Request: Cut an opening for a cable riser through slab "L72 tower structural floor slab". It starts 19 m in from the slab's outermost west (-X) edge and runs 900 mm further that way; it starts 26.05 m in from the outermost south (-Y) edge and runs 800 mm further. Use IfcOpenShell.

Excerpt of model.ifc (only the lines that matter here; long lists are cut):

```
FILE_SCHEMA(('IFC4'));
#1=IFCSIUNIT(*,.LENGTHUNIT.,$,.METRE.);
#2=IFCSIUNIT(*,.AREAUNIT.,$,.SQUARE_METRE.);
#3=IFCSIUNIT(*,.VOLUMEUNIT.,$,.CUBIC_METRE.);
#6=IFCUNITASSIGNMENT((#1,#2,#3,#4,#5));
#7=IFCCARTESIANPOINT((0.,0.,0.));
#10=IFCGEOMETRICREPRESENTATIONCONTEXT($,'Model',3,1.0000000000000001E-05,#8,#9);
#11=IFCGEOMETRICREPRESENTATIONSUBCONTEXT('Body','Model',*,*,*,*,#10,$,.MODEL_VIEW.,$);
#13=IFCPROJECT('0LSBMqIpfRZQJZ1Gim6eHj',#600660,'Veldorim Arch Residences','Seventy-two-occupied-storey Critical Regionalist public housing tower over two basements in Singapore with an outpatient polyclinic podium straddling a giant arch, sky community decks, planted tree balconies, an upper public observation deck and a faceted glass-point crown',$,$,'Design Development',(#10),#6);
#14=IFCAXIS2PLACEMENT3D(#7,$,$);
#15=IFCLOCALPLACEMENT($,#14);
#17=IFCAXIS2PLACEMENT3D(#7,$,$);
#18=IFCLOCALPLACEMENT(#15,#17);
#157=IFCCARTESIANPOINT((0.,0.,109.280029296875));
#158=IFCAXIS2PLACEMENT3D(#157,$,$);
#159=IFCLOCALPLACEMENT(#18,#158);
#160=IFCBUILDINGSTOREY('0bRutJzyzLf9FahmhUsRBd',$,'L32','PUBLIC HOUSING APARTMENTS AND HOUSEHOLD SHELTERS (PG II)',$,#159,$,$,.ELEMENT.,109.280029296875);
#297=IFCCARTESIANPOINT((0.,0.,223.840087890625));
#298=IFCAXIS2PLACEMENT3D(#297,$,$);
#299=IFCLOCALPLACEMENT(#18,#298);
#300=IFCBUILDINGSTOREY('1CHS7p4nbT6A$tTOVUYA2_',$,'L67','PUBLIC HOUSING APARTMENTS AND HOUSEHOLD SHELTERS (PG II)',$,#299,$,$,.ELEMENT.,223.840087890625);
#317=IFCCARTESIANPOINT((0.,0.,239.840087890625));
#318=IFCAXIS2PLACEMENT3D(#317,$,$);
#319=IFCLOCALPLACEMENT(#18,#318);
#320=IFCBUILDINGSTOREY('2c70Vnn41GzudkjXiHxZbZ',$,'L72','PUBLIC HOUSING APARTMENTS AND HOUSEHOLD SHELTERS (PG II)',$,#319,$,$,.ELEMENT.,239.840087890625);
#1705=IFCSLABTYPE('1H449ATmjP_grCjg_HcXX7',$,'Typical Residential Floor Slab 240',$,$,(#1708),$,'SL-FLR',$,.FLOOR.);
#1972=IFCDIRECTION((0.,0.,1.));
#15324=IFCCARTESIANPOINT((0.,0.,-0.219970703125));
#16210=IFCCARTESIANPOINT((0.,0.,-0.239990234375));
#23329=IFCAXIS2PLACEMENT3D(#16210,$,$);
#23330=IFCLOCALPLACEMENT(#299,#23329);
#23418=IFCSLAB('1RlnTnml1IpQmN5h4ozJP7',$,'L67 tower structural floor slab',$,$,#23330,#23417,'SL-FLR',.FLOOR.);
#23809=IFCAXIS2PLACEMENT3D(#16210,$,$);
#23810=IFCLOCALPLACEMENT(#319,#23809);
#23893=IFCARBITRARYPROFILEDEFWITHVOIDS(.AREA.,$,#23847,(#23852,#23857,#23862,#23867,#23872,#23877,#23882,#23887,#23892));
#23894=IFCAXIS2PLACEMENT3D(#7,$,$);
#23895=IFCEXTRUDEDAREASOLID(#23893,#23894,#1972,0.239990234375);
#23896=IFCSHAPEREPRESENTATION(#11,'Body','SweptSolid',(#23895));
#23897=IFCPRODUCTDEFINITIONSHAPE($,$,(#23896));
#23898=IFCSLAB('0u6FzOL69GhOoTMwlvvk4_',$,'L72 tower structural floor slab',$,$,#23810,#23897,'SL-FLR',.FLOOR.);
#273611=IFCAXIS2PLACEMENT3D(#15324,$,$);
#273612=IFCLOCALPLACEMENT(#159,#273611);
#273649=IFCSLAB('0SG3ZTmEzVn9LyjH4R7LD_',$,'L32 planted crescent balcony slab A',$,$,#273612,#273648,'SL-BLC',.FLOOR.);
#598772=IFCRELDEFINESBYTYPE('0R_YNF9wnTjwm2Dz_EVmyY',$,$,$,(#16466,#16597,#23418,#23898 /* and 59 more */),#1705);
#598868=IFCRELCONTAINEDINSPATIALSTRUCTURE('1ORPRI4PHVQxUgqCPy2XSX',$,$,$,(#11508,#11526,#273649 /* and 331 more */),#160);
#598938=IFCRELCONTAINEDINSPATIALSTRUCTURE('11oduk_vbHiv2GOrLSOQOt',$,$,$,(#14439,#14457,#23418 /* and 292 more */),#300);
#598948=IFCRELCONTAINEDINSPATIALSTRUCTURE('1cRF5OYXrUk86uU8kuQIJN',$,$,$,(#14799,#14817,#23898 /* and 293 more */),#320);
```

```python
import numpy as np
import ifcopenshell
import ifcopenshell.api.feature
import ifcopenshell.api.geometry
import ifcopenshell.api.root
import ifcopenshell.geom
import ifcopenshell.util.placement
import ifcopenshell.util.representation
import ifcopenshell.util.shape
import ifcopenshell.util.unit

model = ifcopenshell.open("model.ifc")
unit_scale = ifcopenshell.util.unit.calculate_unit_scale(model)
settings = ifcopenshell.geom.settings()


def volume(element):
    """Net volume in cubic metres, openings subtracted."""
    shape = ifcopenshell.geom.create_shape(settings, element)
    return ifcopenshell.util.shape.get_volume(shape.geometry)


slab = model.by_guid("0u6FzOL69GhOoTMwlvvk4_")
before = volume(slab)

# Extent in the slab's own axes, in metres. The edges named are its -X and -Y sides.
slab_shape = ifcopenshell.geom.create_shape(settings, slab)
vertices = ifcopenshell.util.shape.get_vertices(slab_shape.geometry)
x_min, y_min, bottom = vertices.min(axis=0)
top = vertices[:, 2].max()

opening = ifcopenshell.api.root.create_entity(model, ifc_class="IfcOpeningElement", name="Cable riser opening", predefined_type="OPENING")
context = ifcopenshell.util.representation.get_context(model, "Model", "Body", "MODEL_VIEW")
width, depth = 0.9, 0.8
outline = [(0.0, 0.0), (width, 0.0), (width, depth), (0.0, depth), (0.0, 0.0)]
# Overshoot both faces by 50 mm so the cut is clean.
shape = ifcopenshell.api.geometry.add_slab_representation(
    model, context=context, depth=top - bottom + 0.1, polyline=outline
)
ifcopenshell.api.geometry.assign_representation(model, product=opening, representation=shape)

matrix = ifcopenshell.util.placement.get_local_placement(slab.ObjectPlacement)
matrix[:, 3] = matrix @ np.append(np.array([x_min + 19, y_min + 26.05, bottom - 0.05]) / unit_scale, 1.0)
ifcopenshell.api.geometry.edit_object_placement(model, product=opening, matrix=matrix, is_si=False)
ifcopenshell.api.feature.add_feature(model, feature=opening, element=slab)

after = volume(slab)

print(f"slab volume {before:.3f} -> {after:.3f} m3")

model.write("model_edited.ifc")
```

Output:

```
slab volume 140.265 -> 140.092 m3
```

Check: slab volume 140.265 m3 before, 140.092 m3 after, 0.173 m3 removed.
